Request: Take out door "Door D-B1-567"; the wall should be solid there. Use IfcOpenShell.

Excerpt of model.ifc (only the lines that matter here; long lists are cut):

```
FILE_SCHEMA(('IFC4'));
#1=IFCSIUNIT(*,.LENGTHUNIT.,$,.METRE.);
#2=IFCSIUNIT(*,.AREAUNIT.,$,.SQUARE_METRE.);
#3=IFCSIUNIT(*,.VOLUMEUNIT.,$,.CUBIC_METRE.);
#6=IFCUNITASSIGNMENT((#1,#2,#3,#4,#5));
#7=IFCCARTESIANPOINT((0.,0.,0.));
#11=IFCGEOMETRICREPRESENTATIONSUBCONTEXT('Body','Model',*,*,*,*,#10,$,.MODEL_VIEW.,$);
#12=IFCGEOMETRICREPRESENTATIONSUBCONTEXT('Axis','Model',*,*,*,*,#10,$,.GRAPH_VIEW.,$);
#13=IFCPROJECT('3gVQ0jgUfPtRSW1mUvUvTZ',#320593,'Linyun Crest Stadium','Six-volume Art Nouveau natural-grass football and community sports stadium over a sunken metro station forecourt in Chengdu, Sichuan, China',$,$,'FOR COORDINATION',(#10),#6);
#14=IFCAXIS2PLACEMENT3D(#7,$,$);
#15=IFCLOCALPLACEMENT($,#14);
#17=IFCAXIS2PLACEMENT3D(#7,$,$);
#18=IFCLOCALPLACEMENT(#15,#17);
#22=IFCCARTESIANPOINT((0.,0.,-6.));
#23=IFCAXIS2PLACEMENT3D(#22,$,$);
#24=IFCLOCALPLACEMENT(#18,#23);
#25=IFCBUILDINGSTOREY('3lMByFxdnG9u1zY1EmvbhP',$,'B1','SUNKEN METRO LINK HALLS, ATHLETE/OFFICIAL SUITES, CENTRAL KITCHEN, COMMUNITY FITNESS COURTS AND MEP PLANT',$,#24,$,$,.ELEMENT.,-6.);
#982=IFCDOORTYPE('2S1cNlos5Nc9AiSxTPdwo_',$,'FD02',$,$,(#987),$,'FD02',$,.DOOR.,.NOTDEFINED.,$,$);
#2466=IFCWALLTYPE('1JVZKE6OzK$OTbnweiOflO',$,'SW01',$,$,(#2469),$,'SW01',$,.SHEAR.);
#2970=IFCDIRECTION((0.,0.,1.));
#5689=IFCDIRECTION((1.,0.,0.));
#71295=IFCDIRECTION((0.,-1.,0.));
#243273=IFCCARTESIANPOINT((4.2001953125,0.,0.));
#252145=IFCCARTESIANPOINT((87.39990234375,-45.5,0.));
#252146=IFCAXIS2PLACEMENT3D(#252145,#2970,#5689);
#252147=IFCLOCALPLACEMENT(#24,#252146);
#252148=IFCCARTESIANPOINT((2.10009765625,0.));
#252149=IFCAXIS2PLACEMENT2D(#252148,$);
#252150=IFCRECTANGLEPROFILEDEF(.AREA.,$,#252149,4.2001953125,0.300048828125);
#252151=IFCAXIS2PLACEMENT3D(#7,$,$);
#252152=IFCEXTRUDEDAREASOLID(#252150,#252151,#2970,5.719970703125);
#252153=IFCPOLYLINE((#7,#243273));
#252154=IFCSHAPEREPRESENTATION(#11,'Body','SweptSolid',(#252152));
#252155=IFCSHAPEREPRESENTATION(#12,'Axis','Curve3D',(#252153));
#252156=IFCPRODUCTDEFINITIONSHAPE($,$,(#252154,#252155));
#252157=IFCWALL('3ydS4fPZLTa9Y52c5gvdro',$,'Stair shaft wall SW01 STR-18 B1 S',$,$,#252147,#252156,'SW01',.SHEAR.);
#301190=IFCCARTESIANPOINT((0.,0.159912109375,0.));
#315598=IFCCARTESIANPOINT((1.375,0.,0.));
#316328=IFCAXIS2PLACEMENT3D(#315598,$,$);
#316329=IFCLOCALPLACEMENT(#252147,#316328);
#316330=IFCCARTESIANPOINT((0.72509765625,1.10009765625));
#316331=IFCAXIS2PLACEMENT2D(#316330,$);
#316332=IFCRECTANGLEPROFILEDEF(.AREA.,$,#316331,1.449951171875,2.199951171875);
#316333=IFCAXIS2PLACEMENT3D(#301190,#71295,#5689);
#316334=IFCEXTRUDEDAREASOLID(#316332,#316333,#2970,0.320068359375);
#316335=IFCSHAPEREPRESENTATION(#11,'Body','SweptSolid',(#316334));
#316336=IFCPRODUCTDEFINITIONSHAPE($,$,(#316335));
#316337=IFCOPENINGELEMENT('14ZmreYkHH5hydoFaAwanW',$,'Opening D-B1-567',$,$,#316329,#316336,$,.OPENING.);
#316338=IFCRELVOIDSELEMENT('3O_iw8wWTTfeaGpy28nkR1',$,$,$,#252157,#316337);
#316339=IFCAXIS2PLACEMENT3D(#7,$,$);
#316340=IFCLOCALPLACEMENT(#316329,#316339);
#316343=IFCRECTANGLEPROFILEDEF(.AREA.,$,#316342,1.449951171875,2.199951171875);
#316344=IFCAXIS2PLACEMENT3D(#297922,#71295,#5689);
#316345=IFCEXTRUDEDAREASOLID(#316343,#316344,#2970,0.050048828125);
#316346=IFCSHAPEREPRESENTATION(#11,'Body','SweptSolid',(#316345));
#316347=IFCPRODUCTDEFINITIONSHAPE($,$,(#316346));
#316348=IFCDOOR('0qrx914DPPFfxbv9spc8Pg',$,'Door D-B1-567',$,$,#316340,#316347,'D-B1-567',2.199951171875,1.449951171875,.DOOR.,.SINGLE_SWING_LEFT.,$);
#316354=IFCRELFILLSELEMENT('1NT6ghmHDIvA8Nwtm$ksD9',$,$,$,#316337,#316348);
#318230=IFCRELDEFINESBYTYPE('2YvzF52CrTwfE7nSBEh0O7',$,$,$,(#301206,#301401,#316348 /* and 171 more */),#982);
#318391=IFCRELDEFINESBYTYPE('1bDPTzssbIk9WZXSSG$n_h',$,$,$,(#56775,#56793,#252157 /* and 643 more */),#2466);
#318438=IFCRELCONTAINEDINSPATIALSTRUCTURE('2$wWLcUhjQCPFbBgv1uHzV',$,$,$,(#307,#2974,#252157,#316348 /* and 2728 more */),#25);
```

```python
import ifcopenshell
import ifcopenshell.api.feature
import ifcopenshell.api.root
import ifcopenshell.geom
import ifcopenshell.util.shape

model = ifcopenshell.open("model.ifc")
settings = ifcopenshell.geom.settings()


def volume(element):
    """Net volume in cubic metres, openings subtracted."""
    shape = ifcopenshell.geom.create_shape(settings, element)
    return ifcopenshell.util.shape.get_volume(shape.geometry)


door = model.by_guid("0qrx914DPPFfxbv9spc8Pg")
opening = door.FillsVoids[0].RelatingOpeningElement
wall = opening.VoidsElements[0].RelatingBuildingElement
before = volume(wall)

ifcopenshell.api.root.remove_product(model, product=door)
ifcopenshell.api.feature.remove_feature(model, feature=opening)

after = volume(wall)

print(f"wall volume {before:.3f} -> {after:.3f} m3")

model.write("model-out.ifc")
```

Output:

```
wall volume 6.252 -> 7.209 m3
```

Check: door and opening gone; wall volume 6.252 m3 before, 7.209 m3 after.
